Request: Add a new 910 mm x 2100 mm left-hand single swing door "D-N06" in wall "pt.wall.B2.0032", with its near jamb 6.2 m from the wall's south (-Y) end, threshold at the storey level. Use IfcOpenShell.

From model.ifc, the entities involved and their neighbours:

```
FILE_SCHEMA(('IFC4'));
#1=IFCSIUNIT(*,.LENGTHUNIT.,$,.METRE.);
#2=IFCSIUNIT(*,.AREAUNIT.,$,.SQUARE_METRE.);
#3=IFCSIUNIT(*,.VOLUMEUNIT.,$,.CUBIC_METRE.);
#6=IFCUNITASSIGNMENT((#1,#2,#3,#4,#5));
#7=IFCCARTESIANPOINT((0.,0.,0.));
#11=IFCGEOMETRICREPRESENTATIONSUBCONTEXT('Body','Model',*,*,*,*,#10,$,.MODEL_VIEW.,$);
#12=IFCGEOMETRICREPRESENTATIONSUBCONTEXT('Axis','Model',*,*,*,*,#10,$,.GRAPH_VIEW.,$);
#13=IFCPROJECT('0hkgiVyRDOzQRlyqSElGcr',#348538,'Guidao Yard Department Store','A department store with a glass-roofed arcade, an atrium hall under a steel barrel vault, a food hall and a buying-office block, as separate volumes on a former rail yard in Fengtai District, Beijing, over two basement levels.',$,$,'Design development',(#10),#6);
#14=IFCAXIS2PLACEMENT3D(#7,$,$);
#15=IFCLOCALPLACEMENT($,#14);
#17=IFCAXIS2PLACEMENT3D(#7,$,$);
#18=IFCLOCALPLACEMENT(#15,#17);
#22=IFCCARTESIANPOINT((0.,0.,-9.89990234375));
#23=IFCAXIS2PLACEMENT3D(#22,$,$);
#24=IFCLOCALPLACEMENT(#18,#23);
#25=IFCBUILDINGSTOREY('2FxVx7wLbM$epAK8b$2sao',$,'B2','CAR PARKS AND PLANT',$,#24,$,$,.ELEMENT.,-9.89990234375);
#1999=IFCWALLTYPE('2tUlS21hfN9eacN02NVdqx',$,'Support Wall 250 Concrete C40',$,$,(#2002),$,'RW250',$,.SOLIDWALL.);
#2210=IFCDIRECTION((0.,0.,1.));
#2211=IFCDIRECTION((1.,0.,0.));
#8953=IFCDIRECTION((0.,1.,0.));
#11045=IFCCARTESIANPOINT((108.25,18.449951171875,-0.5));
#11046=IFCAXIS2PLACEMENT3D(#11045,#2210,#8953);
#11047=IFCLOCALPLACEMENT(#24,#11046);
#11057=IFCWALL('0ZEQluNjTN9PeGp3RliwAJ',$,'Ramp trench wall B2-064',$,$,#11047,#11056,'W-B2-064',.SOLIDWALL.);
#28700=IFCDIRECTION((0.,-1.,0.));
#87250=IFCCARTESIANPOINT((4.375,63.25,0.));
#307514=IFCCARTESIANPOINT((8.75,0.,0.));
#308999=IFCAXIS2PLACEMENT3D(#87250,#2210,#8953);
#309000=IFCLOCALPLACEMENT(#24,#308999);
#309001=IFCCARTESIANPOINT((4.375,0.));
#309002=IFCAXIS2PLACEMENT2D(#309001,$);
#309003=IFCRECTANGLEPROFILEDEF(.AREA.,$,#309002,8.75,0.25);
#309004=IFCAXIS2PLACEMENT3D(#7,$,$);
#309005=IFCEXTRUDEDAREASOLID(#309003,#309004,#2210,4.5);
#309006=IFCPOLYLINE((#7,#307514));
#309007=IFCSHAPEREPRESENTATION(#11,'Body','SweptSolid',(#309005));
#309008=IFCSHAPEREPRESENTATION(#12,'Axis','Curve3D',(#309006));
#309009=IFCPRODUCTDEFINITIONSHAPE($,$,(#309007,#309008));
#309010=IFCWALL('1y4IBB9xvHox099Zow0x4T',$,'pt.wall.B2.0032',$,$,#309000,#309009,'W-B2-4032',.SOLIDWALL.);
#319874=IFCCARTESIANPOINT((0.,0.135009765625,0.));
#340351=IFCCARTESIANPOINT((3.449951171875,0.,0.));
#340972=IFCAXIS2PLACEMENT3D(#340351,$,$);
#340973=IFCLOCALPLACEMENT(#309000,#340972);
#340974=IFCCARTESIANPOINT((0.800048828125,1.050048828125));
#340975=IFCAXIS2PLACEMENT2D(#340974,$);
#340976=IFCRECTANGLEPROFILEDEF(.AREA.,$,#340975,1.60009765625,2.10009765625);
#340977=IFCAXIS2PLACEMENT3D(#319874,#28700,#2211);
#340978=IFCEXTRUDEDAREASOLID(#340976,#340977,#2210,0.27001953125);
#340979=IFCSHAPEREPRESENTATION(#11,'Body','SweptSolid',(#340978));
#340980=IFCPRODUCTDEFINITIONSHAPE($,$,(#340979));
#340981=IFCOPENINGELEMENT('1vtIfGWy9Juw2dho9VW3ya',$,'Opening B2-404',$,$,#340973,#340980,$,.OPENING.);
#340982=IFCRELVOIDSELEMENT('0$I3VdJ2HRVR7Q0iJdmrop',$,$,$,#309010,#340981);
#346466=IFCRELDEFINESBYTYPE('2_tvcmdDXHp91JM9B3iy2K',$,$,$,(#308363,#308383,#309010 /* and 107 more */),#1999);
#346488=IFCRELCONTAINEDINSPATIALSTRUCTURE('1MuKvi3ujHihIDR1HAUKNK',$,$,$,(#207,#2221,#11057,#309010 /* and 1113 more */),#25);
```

```python
import numpy as np
import ifcopenshell
import ifcopenshell.api.feature
import ifcopenshell.api.geometry
import ifcopenshell.api.root
import ifcopenshell.api.spatial
import ifcopenshell.geom
import ifcopenshell.util.element
import ifcopenshell.util.placement
import ifcopenshell.util.representation
import ifcopenshell.util.shape
import ifcopenshell.util.unit

model = ifcopenshell.open("model.ifc")
unit_scale = ifcopenshell.util.unit.calculate_unit_scale(model)
settings = ifcopenshell.geom.settings()


def volume(element):
    """Net volume in cubic metres, openings subtracted."""
    shape = ifcopenshell.geom.create_shape(settings, element)
    return ifcopenshell.util.shape.get_volume(shape.geometry)


wall = model.by_id(309010)
storey = ifcopenshell.util.element.get_container(wall, ifc_class="IfcBuildingStorey")
context = ifcopenshell.util.representation.get_context(model, "Model", "Body", "MODEL_VIEW")
before = volume(wall)

width, height, from_end, sill = 0.91, 2.1, 6.2, 0.0  # metres

# The wall runs along its own X axis, and the end named is its -X end.
wall_shape = ifcopenshell.geom.create_shape(settings, wall)
x, y, z = ifcopenshell.util.shape.get_vertices(wall_shape.geometry).T
start = x.min() + from_end
face, thickness = float(y.min()), float(y.max() - y.min())
wall_matrix = ifcopenshell.util.placement.get_local_placement(wall.ObjectPlacement)
level = ifcopenshell.util.placement.get_local_placement(storey.ObjectPlacement)[2, 3]


def in_wall(x, y):
    """Placement at x, y metres in the wall's axes, at sill height."""
    matrix = wall_matrix.copy()
    matrix[:, 3] = wall_matrix @ np.array([x / unit_scale, y / unit_scale, 0.0, 1.0])
    matrix[2, 3] = level + sill / unit_scale
    return matrix


# Opening: a box that overshoots both wall faces by 50 mm.
opening = ifcopenshell.api.root.create_entity(model, ifc_class="IfcOpeningElement", predefined_type="OPENING")
box = ifcopenshell.api.geometry.add_wall_representation(
    model, context=context, length=width, height=height, thickness=thickness + 0.1
)
ifcopenshell.api.geometry.assign_representation(model, product=opening, representation=box)
ifcopenshell.api.geometry.edit_object_placement(model, product=opening, matrix=in_wall(start, face - 0.05), is_si=False)
ifcopenshell.api.feature.add_feature(model, feature=opening, element=wall)

door = ifcopenshell.api.root.create_entity(model, ifc_class="IfcDoor", name="D-N06", predefined_type="DOOR")
door.OverallWidth, door.OverallHeight = width / unit_scale, height / unit_scale
door.OperationType = "SINGLE_SWING_LEFT"
body = ifcopenshell.api.geometry.add_door_representation(
    model,
    context=context,
    overall_width=door.OverallWidth,
    overall_height=door.OverallHeight,
    operation_type="SINGLE_SWING_LEFT",
    lining_properties={"LiningDepth": thickness / unit_scale, "ThresholdDepth": thickness / unit_scale},
)
ifcopenshell.api.geometry.assign_representation(model, product=door, representation=body)
ifcopenshell.api.spatial.assign_container(model, products=[door], relating_structure=storey)
ifcopenshell.api.feature.add_filling(model, opening=opening, element=door)

# The lining spans the wall, so the door starts at the wall face.
ifcopenshell.api.geometry.edit_object_placement(model, product=door, matrix=in_wall(start, face), is_si=False)

after = volume(wall)

print(f"wall volume {before:.3f} -> {after:.3f} m3")

model.write("model_rev.ifc")
```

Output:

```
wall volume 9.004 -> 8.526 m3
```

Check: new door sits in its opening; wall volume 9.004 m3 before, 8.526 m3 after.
